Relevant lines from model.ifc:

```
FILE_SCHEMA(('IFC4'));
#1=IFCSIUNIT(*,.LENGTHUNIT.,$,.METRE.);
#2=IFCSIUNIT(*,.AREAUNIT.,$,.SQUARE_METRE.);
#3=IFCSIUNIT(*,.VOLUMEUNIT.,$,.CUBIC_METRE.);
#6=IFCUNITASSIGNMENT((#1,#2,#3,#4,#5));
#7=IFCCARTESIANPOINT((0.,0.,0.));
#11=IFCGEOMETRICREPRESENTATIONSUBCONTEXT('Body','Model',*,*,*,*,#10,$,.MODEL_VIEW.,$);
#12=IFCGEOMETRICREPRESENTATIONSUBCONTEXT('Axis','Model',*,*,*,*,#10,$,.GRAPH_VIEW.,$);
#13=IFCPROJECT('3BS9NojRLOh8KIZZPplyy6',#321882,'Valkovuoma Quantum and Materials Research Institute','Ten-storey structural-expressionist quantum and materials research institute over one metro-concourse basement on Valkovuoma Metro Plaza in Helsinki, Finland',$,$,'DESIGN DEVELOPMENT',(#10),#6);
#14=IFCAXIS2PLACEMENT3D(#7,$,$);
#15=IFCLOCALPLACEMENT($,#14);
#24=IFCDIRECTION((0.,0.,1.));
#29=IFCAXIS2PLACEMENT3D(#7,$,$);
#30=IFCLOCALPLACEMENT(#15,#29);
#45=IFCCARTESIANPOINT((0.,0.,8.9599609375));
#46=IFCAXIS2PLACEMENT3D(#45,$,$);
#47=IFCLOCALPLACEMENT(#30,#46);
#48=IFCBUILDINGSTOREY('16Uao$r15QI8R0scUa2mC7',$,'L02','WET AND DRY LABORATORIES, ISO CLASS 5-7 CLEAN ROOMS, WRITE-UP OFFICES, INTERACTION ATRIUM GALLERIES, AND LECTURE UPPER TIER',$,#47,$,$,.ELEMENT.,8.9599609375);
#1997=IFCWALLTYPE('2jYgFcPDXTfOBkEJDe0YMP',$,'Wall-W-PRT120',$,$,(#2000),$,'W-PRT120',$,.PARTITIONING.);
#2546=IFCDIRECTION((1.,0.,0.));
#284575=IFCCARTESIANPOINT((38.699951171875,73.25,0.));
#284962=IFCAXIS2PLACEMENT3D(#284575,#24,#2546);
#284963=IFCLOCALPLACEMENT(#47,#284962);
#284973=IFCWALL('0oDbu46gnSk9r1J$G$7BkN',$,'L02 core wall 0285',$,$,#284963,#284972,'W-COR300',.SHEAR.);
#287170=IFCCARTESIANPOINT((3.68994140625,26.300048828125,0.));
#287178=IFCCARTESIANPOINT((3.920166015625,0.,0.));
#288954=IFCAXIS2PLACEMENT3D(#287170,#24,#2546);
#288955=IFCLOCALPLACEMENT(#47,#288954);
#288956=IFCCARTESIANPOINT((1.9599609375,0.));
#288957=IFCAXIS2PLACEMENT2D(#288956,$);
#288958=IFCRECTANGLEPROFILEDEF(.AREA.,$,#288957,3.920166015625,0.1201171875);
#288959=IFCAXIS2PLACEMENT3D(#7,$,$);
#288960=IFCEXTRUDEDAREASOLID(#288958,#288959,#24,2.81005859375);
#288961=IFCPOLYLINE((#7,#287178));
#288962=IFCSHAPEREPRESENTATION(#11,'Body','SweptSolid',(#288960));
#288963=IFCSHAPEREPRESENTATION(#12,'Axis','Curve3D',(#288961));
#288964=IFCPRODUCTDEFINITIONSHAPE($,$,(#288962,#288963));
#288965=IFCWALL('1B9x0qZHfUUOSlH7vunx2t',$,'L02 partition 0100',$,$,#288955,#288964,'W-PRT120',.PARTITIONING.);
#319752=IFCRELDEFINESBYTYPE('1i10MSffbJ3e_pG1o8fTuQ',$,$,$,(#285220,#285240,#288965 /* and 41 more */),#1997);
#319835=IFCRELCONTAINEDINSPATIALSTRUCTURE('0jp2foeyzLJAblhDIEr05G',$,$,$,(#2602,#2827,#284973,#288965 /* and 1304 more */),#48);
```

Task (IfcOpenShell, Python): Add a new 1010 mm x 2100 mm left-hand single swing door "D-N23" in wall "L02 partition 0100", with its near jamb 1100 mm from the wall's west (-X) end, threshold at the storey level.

```python
import numpy as np
import ifcopenshell
import ifcopenshell.api.feature
import ifcopenshell.api.geometry
import ifcopenshell.api.root
import ifcopenshell.api.spatial
import ifcopenshell.geom
import ifcopenshell.util.element
import ifcopenshell.util.placement
import ifcopenshell.util.representation
import ifcopenshell.util.shape
import ifcopenshell.util.unit

model = ifcopenshell.open("model.ifc")
unit_scale = ifcopenshell.util.unit.calculate_unit_scale(model)
settings = ifcopenshell.geom.settings()


def volume(element):
    """Net volume in cubic metres, openings subtracted."""
    shape = ifcopenshell.geom.create_shape(settings, element)
    return ifcopenshell.util.shape.get_volume(shape.geometry)


wall = model.by_guid("1B9x0qZHfUUOSlH7vunx2t")
storey = ifcopenshell.util.element.get_container(wall, ifc_class="IfcBuildingStorey")
context = ifcopenshell.util.representation.get_context(model, "Model", "Body", "MODEL_VIEW")
before = volume(wall)

width, height, from_end, sill = 1.01, 2.1, 1.1, 0.0  # metres

# The wall runs along its own X axis, and the end named is its -X end.
wall_shape = ifcopenshell.geom.create_shape(settings, wall)
x, y, z = ifcopenshell.util.shape.get_vertices(wall_shape.geometry).T
start = x.min() + from_end
face, thickness = float(y.min()), float(y.max() - y.min())
wall_matrix = ifcopenshell.util.placement.get_local_placement(wall.ObjectPlacement)
level = ifcopenshell.util.placement.get_local_placement(storey.ObjectPlacement)[2, 3]


def in_wall(x, y):
    """Placement at x, y metres in the wall's axes, at sill height."""
    matrix = wall_matrix.copy()
    matrix[:, 3] = wall_matrix @ np.array([x / unit_scale, y / unit_scale, 0.0, 1.0])
    matrix[2, 3] = level + sill / unit_scale
    return matrix


# Opening: a box that overshoots both wall faces by 50 mm.
opening = ifcopenshell.api.root.create_entity(model, ifc_class="IfcOpeningElement", predefined_type="OPENING")
box = ifcopenshell.api.geometry.add_wall_representation(
    model, context=context, length=width, height=height, thickness=thickness + 0.1
)
ifcopenshell.api.geometry.assign_representation(model, product=opening, representation=box)
ifcopenshell.api.geometry.edit_object_placement(model, product=opening, matrix=in_wall(start, face - 0.05), is_si=False)
ifcopenshell.api.feature.add_feature(model, feature=opening, element=wall)

door = ifcopenshell.api.root.create_entity(model, ifc_class="IfcDoor", name="D-N23", predefined_type="DOOR")
door.OverallWidth, door.OverallHeight = width / unit_scale, height / unit_scale
door.OperationType = "SINGLE_SWING_LEFT"
body = ifcopenshell.api.geometry.add_door_representation(
    model,
    context=context,
    overall_width=door.OverallWidth,
    overall_height=door.OverallHeight,
    operation_type="SINGLE_SWING_LEFT",
    lining_properties={"LiningDepth": thickness / unit_scale, "ThresholdDepth": thickness / unit_scale},
)
ifcopenshell.api.geometry.assign_representation(model, product=door, representation=body)
ifcopenshell.api.spatial.assign_container(model, products=[door], relating_structure=storey)
ifcopenshell.api.feature.add_filling(model, opening=opening, element=door)

# The lining spans the wall, so the door starts at the wall face.
ifcopenshell.api.geometry.edit_object_placement(model, product=door, matrix=in_wall(start, face), is_si=False)

after = volume(wall)

print(f"wall volume {before:.3f} -> {after:.3f} m3")

model.write("model_updated.ifc")
```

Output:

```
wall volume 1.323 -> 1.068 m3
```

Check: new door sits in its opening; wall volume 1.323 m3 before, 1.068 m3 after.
